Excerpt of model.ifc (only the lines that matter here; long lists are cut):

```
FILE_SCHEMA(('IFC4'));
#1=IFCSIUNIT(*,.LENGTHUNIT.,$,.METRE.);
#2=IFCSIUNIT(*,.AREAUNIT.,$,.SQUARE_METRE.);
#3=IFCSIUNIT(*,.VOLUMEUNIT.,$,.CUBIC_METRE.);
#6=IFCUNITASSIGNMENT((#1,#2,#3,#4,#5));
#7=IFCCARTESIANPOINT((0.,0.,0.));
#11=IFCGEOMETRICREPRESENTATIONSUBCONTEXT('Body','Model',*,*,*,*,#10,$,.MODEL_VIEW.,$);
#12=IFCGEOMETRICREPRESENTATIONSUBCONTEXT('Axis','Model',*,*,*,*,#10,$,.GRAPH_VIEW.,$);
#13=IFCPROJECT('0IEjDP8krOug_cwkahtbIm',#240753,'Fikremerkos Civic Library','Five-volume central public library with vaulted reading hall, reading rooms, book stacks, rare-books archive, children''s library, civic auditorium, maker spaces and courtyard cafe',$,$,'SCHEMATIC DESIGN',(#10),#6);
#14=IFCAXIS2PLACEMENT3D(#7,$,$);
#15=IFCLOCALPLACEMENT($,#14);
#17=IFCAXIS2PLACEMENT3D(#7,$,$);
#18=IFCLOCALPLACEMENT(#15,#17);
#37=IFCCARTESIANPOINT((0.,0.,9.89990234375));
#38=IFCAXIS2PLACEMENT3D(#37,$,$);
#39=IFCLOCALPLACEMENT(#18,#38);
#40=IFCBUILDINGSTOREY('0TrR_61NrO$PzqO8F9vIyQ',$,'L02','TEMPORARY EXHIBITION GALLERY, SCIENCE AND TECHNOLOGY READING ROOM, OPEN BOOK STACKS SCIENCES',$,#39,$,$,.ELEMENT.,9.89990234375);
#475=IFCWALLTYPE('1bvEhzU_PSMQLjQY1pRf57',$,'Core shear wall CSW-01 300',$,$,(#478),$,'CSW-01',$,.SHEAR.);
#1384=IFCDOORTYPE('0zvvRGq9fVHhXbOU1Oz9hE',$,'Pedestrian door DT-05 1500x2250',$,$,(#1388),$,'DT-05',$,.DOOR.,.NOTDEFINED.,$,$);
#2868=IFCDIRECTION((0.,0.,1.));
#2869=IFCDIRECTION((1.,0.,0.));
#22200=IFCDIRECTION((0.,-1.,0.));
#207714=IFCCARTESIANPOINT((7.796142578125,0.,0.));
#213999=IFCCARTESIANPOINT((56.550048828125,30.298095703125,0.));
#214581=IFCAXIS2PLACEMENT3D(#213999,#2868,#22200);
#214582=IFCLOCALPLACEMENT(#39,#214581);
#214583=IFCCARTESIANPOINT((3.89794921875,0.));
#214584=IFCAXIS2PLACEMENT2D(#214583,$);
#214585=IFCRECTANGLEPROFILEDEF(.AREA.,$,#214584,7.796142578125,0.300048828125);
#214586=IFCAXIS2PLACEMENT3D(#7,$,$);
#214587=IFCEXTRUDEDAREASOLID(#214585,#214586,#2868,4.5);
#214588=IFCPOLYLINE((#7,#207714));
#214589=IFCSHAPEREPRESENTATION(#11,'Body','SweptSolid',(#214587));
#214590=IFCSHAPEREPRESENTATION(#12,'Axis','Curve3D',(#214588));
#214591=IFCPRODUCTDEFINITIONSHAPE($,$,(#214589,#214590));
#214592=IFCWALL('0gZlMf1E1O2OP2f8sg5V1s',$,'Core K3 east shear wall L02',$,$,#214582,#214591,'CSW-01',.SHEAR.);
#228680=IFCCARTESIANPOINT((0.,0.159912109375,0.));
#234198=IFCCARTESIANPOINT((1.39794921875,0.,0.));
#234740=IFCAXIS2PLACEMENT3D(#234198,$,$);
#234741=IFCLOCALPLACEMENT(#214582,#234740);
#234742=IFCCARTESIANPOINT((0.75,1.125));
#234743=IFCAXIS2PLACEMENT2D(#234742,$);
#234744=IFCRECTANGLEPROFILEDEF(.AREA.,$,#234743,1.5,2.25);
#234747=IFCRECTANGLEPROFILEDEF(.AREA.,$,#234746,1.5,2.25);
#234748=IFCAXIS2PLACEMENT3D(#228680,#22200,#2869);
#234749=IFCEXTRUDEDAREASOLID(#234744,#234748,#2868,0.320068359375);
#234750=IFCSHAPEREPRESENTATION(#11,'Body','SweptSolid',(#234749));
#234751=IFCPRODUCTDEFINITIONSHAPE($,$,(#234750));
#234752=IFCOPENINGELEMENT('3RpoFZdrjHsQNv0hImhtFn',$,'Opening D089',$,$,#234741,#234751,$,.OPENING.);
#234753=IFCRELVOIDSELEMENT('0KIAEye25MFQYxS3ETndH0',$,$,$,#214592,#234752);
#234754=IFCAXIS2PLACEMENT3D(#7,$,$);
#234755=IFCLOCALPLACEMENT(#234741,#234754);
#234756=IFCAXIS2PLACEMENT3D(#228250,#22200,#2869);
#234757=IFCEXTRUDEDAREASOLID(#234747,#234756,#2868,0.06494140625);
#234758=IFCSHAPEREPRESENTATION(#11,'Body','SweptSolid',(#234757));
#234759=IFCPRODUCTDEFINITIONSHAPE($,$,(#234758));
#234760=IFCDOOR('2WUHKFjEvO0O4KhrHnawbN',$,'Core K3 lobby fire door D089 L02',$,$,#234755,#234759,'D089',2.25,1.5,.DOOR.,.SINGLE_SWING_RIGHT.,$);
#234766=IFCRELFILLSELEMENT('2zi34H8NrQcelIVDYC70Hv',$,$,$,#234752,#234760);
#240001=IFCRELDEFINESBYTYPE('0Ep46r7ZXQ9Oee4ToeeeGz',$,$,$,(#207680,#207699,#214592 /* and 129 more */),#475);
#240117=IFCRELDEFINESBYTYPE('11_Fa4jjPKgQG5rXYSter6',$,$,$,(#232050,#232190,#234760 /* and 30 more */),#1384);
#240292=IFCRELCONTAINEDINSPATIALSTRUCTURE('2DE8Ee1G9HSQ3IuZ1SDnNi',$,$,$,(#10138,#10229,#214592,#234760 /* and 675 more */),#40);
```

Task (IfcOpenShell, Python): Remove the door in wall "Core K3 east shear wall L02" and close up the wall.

```python
import ifcopenshell
import ifcopenshell.api.feature
import ifcopenshell.api.root
import ifcopenshell.geom
import ifcopenshell.util.shape

model = ifcopenshell.open("model.ifc")
settings = ifcopenshell.geom.settings()


def volume(element):
    """Net volume in cubic metres, openings subtracted."""
    shape = ifcopenshell.geom.create_shape(settings, element)
    return ifcopenshell.util.shape.get_volume(shape.geometry)


door = model.by_guid("2WUHKFjEvO0O4KhrHnawbN")
opening = door.FillsVoids[0].RelatingOpeningElement
wall = opening.VoidsElements[0].RelatingBuildingElement
before = volume(wall)

ifcopenshell.api.root.remove_product(model, product=door)
ifcopenshell.api.feature.remove_feature(model, feature=opening)

after = volume(wall)

print(f"wall volume {before:.3f} -> {after:.3f} m3")

model.write("model_updated.ifc")
```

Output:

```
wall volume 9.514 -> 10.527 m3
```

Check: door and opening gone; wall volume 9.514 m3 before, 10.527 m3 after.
